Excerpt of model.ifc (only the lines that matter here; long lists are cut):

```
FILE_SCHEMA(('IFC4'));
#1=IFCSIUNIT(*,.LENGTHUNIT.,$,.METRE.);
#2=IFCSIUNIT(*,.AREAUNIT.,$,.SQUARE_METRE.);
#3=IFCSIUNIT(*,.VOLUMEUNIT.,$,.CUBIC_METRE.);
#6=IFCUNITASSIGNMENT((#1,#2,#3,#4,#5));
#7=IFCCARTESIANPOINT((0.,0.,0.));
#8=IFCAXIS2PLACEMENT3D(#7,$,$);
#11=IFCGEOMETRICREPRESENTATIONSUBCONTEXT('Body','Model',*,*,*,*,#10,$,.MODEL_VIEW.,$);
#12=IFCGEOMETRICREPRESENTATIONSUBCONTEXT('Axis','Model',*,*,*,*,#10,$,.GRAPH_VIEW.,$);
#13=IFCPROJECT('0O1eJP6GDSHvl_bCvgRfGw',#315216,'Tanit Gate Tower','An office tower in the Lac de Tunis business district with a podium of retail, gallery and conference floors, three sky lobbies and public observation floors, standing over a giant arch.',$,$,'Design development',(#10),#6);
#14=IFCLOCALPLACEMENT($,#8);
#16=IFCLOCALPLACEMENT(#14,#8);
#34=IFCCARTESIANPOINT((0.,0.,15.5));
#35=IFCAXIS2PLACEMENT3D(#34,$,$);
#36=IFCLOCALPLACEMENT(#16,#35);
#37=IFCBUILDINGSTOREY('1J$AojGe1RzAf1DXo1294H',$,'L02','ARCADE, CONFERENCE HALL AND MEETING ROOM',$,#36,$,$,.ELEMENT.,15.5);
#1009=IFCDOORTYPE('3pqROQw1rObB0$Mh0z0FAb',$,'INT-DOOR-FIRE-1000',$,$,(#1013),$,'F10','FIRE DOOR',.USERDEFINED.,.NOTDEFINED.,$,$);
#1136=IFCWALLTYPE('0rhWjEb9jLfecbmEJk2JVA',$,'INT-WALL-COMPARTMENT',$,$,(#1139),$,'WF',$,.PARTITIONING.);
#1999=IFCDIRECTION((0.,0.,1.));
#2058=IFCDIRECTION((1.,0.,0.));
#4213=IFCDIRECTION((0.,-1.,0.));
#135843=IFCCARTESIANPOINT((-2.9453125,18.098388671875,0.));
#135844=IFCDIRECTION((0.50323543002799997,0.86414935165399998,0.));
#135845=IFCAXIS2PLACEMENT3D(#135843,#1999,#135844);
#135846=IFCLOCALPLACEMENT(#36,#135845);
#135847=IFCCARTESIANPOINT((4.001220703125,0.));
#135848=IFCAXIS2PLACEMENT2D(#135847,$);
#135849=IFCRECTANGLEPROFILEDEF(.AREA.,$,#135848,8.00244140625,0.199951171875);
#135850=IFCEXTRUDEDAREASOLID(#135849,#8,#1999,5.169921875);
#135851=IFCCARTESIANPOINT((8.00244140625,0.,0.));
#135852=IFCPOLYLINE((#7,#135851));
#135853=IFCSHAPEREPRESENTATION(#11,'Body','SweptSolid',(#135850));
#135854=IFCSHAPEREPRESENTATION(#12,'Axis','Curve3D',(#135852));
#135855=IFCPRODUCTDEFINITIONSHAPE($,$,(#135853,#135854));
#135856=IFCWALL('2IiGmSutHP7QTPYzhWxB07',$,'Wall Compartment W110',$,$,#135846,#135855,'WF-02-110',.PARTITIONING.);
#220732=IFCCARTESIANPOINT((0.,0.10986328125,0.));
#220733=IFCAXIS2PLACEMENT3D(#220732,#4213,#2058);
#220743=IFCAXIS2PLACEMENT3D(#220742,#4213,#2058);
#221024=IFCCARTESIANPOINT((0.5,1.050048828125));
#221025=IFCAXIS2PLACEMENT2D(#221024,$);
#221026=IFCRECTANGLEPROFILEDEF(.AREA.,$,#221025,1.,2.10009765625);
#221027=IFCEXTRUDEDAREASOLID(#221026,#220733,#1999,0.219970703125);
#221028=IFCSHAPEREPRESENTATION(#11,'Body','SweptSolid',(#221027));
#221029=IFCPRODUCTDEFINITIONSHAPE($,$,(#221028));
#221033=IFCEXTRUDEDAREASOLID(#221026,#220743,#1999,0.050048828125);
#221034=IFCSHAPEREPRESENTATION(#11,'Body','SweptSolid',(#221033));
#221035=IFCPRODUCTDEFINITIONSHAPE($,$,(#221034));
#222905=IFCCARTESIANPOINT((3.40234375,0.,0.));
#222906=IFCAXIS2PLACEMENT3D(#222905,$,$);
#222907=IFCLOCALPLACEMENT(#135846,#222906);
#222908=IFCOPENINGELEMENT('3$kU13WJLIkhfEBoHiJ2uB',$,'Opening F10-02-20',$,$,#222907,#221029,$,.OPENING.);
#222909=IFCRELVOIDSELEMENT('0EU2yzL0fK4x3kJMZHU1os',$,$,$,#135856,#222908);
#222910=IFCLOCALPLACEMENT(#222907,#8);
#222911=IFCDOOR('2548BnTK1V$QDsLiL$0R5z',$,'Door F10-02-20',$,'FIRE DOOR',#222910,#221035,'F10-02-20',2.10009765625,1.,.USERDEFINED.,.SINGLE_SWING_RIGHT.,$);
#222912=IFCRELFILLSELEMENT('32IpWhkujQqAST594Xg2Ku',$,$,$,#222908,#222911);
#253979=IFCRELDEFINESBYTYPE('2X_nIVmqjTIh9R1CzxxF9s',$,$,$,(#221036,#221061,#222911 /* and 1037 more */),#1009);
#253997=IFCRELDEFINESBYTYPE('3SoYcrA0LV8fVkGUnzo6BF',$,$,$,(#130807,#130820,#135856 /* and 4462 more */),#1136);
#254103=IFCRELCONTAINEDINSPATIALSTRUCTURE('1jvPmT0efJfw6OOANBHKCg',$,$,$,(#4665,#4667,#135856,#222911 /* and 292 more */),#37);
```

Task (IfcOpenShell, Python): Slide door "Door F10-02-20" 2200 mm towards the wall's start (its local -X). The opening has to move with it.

```python
import ifcopenshell
import ifcopenshell.api.geometry
import ifcopenshell.util.placement
import ifcopenshell.util.unit

model = ifcopenshell.open("model.ifc")
unit_scale = ifcopenshell.util.unit.calculate_unit_scale(model)

door = model.by_guid("2548BnTK1V$QDsLiL$0R5z")
opening = door.FillsVoids[0].RelatingOpeningElement
wall = opening.VoidsElements[0].RelatingBuildingElement

wall_matrix = ifcopenshell.util.placement.get_local_placement(wall.ObjectPlacement)
shift = wall_matrix[:3, 0] * -2.2 / unit_scale
before = ifcopenshell.util.placement.get_local_placement(door.ObjectPlacement)[:3, 3].copy()

# The door is placed relative to its opening, so it follows when the opening moves.
matrix = ifcopenshell.util.placement.get_local_placement(opening.ObjectPlacement)
matrix[:3, 3] += shift
ifcopenshell.api.geometry.edit_object_placement(
    model, product=opening, matrix=matrix, is_si=False, should_transform_children=True
)

after = ifcopenshell.util.placement.get_local_placement(door.ObjectPlacement)[:3, 3]
print("door moved by", (after - before).round(3) + 0.0)

model.write("model_updated.ifc")
```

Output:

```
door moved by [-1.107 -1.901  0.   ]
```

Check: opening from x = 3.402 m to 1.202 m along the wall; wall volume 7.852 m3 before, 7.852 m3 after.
